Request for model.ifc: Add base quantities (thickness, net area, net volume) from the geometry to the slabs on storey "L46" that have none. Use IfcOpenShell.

First a look at what the model holds.

```python
import ifcopenshell
import ifcopenshell.util.element
import ifcopenshell.util.unit

model = ifcopenshell.open("model.ifc")
print(model.schema)
for unit_type in ("LENGTHUNIT", "AREAUNIT", "VOLUMEUNIT"):
    print(unit_type, ifcopenshell.util.unit.calculate_unit_scale(model, unit_type))
storey = next(s for s in model.by_type("IfcBuildingStorey") if s.Name == "L46")
slabs = [e for e in ifcopenshell.util.element.get_decomposition(storey) if e.is_a("IfcSlab")]
for e in sorted(slabs, key=lambda e: e.id()):
    print(e.id(), e.is_a(), e.Name, list(ifcopenshell.util.element.get_psets(e, qtos_only=True)), sep=" | ")
```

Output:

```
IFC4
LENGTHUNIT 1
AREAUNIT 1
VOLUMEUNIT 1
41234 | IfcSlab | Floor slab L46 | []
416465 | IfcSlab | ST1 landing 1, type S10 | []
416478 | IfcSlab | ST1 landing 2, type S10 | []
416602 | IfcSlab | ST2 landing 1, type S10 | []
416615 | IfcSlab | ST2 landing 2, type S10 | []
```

```python
import ifcopenshell
import ifcopenshell.api.pset
import ifcopenshell.geom
import ifcopenshell.util.element
import ifcopenshell.util.shape
import ifcopenshell.util.unit

model = ifcopenshell.open("model.ifc")
unit_scale = ifcopenshell.util.unit.calculate_unit_scale(model)
area_scale = ifcopenshell.util.unit.calculate_unit_scale(model, "AREAUNIT")
volume_scale = ifcopenshell.util.unit.calculate_unit_scale(model, "VOLUMEUNIT")
settings = ifcopenshell.geom.settings()

storey = next(s for s in model.by_type("IfcBuildingStorey") if s.Name == "L46")
slabs = [e for e in ifcopenshell.util.element.get_decomposition(storey) if e.is_a("IfcSlab")]

for e in sorted(slabs, key=lambda e: e.id()):
    if ifcopenshell.util.element.get_psets(e, qtos_only=True, should_inherit=False):
        continue
    # Geometry comes back in metres, in the element's own axes.
    shape = ifcopenshell.geom.create_shape(settings, e)
    values = {
        "Width": ifcopenshell.util.shape.get_z(shape.geometry) / unit_scale,
        "NetArea": ifcopenshell.util.shape.get_footprint_area(shape.geometry) / area_scale,
        "NetVolume": ifcopenshell.util.shape.get_volume(shape.geometry) / volume_scale,
    }
    qto = ifcopenshell.api.pset.add_qto(model, product=e, name="Qto_SlabBaseQuantities")
    ifcopenshell.api.pset.edit_qto(model, qto=qto, properties=values)
    print(e.id(), {k: round(v, 3) for k, v in values.items()})

model.write("model-out.ifc")
```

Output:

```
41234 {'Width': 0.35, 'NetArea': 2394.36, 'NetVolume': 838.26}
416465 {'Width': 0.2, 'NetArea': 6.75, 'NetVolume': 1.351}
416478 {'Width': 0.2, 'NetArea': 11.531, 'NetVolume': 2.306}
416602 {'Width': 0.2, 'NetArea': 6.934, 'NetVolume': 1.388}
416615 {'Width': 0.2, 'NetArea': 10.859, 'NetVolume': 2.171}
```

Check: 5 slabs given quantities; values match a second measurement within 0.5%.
